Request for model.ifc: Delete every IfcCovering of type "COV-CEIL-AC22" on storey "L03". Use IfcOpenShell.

First a look at what the model holds.

```python
import ifcopenshell
import ifcopenshell.util.element

model = ifcopenshell.open("model.ifc")
print(model.schema)
storey = next(s for s in model.by_type("IfcBuildingStorey") if s.Name == "L03")
coverings = [e for e in ifcopenshell.util.element.get_decomposition(storey) if e.is_a("IfcCovering")]
seen = {}
for e in coverings:
    element_type = ifcopenshell.util.element.get_type(e)
    name = element_type.Name if element_type not in (None, e) else None
    seen[name] = seen.get(name, 0) + 1
for name, count in sorted(seen.items(), key=str):
    print(count, "x", name)
```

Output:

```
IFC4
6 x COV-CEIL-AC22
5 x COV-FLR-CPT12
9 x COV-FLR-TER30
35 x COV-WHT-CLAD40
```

```python
import ifcopenshell
import ifcopenshell.api.root
import ifcopenshell.util.element

model = ifcopenshell.open("model.ifc")

storey = next(s for s in model.by_type("IfcBuildingStorey") if s.Name == "L03")
coverings = [e for e in ifcopenshell.util.element.get_decomposition(storey) if e.is_a("IfcCovering")]
targets = [e for e in coverings if (t := ifcopenshell.util.element.get_type(e)) not in (None, e) and t.Name == "COV-CEIL-AC22"]

for e in targets:
    ifcopenshell.api.root.remove_product(model, product=e)
print(len(targets), "removed")

model.write("model-out.ifc")
```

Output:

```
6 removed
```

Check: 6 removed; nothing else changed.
